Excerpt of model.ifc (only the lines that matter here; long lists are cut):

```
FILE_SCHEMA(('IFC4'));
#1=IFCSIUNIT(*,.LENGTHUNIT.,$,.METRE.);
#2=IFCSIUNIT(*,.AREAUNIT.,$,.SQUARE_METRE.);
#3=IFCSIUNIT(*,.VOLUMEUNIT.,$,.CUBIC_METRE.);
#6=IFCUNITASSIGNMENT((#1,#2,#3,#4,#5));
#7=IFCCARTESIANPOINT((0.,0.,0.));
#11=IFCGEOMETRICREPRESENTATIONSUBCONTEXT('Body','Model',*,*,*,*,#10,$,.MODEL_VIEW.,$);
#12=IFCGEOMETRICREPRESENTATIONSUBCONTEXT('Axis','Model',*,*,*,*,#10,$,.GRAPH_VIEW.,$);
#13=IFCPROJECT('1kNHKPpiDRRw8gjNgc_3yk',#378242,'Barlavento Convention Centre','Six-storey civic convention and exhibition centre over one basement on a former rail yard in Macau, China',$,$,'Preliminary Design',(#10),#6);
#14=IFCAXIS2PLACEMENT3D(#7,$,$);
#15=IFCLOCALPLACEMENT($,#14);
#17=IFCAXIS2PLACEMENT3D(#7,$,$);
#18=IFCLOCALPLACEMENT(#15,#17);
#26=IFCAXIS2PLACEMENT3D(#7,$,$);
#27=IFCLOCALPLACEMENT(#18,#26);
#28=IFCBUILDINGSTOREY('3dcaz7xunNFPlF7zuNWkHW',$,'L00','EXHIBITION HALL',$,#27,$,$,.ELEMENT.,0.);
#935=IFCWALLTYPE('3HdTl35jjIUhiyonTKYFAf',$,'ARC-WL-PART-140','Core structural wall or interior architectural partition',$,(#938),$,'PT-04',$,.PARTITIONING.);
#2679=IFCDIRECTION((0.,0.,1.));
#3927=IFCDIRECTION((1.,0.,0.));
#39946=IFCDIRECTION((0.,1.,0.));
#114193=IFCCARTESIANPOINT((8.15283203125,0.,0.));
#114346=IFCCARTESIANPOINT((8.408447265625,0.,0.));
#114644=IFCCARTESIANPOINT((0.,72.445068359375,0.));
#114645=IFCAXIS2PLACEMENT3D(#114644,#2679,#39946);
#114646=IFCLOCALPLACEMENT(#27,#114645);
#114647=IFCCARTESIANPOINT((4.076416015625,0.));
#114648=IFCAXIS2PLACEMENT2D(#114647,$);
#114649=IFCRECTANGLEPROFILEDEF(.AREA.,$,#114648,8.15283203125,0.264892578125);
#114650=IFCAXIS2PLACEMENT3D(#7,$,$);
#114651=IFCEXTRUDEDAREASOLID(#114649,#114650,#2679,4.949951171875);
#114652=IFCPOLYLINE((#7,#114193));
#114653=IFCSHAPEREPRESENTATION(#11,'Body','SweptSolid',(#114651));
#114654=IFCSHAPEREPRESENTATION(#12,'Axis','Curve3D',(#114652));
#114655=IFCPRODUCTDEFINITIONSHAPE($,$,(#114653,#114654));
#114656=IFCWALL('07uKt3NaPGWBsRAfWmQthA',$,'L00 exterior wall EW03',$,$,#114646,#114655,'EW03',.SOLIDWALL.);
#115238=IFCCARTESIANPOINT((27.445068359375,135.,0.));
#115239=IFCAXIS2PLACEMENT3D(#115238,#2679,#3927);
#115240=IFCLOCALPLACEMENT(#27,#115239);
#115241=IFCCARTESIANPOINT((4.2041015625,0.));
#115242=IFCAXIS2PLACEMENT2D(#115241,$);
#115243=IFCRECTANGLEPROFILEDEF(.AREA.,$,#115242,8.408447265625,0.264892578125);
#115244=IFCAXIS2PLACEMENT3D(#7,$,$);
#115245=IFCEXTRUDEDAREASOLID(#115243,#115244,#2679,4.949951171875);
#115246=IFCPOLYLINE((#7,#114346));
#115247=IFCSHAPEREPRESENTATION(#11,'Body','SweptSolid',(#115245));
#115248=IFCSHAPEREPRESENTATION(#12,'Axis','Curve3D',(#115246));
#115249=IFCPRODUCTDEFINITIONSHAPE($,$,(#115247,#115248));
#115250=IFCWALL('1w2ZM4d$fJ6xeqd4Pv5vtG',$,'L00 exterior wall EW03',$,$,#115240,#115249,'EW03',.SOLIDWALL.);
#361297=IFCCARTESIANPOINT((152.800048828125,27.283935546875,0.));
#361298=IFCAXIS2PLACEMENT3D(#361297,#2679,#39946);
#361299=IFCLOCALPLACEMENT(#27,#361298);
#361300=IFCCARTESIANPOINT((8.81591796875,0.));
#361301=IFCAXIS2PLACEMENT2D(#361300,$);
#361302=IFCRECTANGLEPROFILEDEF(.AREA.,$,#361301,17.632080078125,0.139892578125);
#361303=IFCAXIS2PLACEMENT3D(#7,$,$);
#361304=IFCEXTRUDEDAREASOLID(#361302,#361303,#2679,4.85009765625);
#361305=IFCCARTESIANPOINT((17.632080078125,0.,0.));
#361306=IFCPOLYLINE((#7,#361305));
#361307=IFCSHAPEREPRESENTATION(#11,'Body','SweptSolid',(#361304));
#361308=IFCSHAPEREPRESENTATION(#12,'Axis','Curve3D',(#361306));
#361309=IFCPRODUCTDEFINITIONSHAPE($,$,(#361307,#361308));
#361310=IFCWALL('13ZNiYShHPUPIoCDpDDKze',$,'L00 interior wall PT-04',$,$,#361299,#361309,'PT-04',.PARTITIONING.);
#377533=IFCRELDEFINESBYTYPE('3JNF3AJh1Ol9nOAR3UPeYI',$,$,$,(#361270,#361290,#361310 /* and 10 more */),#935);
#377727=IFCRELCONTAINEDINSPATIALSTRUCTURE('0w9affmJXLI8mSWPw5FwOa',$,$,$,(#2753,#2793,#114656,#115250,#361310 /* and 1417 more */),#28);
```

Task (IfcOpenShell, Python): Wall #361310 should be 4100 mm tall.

```python
import ifcopenshell
import ifcopenshell.geom
import ifcopenshell.util.representation
import ifcopenshell.util.shape
import ifcopenshell.util.unit

model = ifcopenshell.open("model.ifc")
unit_scale = ifcopenshell.util.unit.calculate_unit_scale(model)
settings = ifcopenshell.geom.settings()


def volume(element):
    """Net volume in cubic metres, openings subtracted."""
    shape = ifcopenshell.geom.create_shape(settings, element)
    return ifcopenshell.util.shape.get_volume(shape.geometry)


wall = model.by_guid("13ZNiYShHPUPIoCDpDDKze")
before = volume(wall)

body = ifcopenshell.util.representation.get_representation(wall, "Model", "Body")
solid = body.Items[0]
old_height = solid.Depth
solid.Depth = 4.1 / unit_scale
after = volume(wall)

print(f"height {old_height:g} -> {solid.Depth:g}, volume {before:.3f} -> {after:.3f} m3")

model.write("model-out.ifc")
```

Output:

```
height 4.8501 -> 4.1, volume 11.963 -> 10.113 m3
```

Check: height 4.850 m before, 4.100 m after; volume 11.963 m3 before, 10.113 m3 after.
